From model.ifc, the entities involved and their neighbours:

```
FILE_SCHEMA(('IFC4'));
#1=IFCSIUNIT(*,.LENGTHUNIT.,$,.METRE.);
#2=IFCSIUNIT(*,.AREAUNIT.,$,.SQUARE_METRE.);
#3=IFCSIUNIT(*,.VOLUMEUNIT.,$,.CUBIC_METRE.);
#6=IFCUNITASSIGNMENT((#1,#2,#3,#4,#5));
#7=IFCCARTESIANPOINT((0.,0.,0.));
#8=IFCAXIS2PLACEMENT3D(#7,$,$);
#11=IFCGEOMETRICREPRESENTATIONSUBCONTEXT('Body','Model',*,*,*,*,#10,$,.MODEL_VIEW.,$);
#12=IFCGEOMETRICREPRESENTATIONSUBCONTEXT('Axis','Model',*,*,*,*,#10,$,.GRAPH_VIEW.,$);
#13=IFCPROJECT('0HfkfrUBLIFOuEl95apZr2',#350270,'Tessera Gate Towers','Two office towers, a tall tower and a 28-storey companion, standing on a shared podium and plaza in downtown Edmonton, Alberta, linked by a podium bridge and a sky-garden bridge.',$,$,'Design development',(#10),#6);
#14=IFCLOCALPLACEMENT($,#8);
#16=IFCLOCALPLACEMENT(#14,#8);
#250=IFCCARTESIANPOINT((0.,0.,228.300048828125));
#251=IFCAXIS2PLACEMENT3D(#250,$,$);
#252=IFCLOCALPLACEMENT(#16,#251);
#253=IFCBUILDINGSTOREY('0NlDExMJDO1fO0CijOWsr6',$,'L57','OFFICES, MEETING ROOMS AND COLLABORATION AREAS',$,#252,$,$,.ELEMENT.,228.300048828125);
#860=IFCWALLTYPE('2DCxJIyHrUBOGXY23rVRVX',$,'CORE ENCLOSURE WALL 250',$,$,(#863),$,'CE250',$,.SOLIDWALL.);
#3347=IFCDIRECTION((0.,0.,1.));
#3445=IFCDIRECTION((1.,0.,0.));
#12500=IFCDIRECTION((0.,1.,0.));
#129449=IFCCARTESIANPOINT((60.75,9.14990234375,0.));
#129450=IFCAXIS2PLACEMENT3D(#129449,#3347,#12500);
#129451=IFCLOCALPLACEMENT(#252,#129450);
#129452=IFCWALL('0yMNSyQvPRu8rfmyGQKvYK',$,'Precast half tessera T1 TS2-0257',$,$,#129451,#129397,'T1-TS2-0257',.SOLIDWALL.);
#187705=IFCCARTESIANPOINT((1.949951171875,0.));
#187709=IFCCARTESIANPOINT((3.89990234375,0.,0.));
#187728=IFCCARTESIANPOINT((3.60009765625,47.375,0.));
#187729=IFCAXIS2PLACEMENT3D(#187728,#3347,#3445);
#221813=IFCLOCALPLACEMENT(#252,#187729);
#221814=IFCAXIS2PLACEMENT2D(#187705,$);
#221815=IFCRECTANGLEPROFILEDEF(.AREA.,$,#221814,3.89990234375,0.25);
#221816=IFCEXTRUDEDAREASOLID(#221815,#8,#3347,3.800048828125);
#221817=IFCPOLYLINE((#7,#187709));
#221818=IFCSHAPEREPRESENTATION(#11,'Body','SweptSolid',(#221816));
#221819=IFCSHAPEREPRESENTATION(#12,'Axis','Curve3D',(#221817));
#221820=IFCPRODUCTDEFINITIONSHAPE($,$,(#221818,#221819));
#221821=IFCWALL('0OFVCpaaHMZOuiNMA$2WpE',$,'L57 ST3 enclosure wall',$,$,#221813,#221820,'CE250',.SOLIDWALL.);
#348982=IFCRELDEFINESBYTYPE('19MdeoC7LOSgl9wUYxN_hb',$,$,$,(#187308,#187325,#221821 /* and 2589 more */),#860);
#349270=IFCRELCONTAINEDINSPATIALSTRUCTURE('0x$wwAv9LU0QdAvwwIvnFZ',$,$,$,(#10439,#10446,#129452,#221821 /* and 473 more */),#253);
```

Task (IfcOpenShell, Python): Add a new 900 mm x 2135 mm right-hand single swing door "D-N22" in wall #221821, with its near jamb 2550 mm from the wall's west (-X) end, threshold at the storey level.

```python
import numpy as np
import ifcopenshell
import ifcopenshell.api.feature
import ifcopenshell.api.geometry
import ifcopenshell.api.root
import ifcopenshell.api.spatial
import ifcopenshell.geom
import ifcopenshell.util.element
import ifcopenshell.util.placement
import ifcopenshell.util.representation
import ifcopenshell.util.shape
import ifcopenshell.util.unit

model = ifcopenshell.open("model.ifc")
unit_scale = ifcopenshell.util.unit.calculate_unit_scale(model)
settings = ifcopenshell.geom.settings()


def volume(element):
    """Net volume in cubic metres, openings subtracted."""
    shape = ifcopenshell.geom.create_shape(settings, element)
    return ifcopenshell.util.shape.get_volume(shape.geometry)


wall = model.by_id(221821)
storey = ifcopenshell.util.element.get_container(wall, ifc_class="IfcBuildingStorey")
context = ifcopenshell.util.representation.get_context(model, "Model", "Body", "MODEL_VIEW")
before = volume(wall)

width, height, from_end, sill = 0.9, 2.135, 2.55, 0.0  # metres

# The wall runs along its own X axis, and the end named is its -X end.
wall_shape = ifcopenshell.geom.create_shape(settings, wall)
x, y, z = ifcopenshell.util.shape.get_vertices(wall_shape.geometry).T
start = x.min() + from_end
face, thickness = float(y.min()), float(y.max() - y.min())
wall_matrix = ifcopenshell.util.placement.get_local_placement(wall.ObjectPlacement)
level = ifcopenshell.util.placement.get_local_placement(storey.ObjectPlacement)[2, 3]


def in_wall(x, y):
    """Placement at x, y metres in the wall's axes, at sill height."""
    matrix = wall_matrix.copy()
    matrix[:, 3] = wall_matrix @ np.array([x / unit_scale, y / unit_scale, 0.0, 1.0])
    matrix[2, 3] = level + sill / unit_scale
    return matrix


# Opening: a box that overshoots both wall faces by 50 mm.
opening = ifcopenshell.api.root.create_entity(model, ifc_class="IfcOpeningElement", predefined_type="OPENING")
box = ifcopenshell.api.geometry.add_wall_representation(
    model, context=context, length=width, height=height, thickness=thickness + 0.1
)
ifcopenshell.api.geometry.assign_representation(model, product=opening, representation=box)
ifcopenshell.api.geometry.edit_object_placement(model, product=opening, matrix=in_wall(start, face - 0.05), is_si=False)
ifcopenshell.api.feature.add_feature(model, feature=opening, element=wall)

door = ifcopenshell.api.root.create_entity(model, ifc_class="IfcDoor", name="D-N22", predefined_type="DOOR")
door.OverallWidth, door.OverallHeight = width / unit_scale, height / unit_scale
door.OperationType = "SINGLE_SWING_RIGHT"
body = ifcopenshell.api.geometry.add_door_representation(
    model,
    context=context,
    overall_width=door.OverallWidth,
    overall_height=door.OverallHeight,
    operation_type="SINGLE_SWING_RIGHT",
    lining_properties={"LiningDepth": thickness / unit_scale, "ThresholdDepth": thickness / unit_scale},
)
ifcopenshell.api.geometry.assign_representation(model, product=door, representation=body)
ifcopenshell.api.spatial.assign_container(model, products=[door], relating_structure=storey)
ifcopenshell.api.feature.add_filling(model, opening=opening, element=door)

# The lining spans the wall, so the door starts at the wall face.
ifcopenshell.api.geometry.edit_object_placement(model, product=door, matrix=in_wall(start, face), is_si=False)

after = volume(wall)

print(f"wall volume {before:.3f} -> {after:.3f} m3")

model.write("model_edited.ifc")
```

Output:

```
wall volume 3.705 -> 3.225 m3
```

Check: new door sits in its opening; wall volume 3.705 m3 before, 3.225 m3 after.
